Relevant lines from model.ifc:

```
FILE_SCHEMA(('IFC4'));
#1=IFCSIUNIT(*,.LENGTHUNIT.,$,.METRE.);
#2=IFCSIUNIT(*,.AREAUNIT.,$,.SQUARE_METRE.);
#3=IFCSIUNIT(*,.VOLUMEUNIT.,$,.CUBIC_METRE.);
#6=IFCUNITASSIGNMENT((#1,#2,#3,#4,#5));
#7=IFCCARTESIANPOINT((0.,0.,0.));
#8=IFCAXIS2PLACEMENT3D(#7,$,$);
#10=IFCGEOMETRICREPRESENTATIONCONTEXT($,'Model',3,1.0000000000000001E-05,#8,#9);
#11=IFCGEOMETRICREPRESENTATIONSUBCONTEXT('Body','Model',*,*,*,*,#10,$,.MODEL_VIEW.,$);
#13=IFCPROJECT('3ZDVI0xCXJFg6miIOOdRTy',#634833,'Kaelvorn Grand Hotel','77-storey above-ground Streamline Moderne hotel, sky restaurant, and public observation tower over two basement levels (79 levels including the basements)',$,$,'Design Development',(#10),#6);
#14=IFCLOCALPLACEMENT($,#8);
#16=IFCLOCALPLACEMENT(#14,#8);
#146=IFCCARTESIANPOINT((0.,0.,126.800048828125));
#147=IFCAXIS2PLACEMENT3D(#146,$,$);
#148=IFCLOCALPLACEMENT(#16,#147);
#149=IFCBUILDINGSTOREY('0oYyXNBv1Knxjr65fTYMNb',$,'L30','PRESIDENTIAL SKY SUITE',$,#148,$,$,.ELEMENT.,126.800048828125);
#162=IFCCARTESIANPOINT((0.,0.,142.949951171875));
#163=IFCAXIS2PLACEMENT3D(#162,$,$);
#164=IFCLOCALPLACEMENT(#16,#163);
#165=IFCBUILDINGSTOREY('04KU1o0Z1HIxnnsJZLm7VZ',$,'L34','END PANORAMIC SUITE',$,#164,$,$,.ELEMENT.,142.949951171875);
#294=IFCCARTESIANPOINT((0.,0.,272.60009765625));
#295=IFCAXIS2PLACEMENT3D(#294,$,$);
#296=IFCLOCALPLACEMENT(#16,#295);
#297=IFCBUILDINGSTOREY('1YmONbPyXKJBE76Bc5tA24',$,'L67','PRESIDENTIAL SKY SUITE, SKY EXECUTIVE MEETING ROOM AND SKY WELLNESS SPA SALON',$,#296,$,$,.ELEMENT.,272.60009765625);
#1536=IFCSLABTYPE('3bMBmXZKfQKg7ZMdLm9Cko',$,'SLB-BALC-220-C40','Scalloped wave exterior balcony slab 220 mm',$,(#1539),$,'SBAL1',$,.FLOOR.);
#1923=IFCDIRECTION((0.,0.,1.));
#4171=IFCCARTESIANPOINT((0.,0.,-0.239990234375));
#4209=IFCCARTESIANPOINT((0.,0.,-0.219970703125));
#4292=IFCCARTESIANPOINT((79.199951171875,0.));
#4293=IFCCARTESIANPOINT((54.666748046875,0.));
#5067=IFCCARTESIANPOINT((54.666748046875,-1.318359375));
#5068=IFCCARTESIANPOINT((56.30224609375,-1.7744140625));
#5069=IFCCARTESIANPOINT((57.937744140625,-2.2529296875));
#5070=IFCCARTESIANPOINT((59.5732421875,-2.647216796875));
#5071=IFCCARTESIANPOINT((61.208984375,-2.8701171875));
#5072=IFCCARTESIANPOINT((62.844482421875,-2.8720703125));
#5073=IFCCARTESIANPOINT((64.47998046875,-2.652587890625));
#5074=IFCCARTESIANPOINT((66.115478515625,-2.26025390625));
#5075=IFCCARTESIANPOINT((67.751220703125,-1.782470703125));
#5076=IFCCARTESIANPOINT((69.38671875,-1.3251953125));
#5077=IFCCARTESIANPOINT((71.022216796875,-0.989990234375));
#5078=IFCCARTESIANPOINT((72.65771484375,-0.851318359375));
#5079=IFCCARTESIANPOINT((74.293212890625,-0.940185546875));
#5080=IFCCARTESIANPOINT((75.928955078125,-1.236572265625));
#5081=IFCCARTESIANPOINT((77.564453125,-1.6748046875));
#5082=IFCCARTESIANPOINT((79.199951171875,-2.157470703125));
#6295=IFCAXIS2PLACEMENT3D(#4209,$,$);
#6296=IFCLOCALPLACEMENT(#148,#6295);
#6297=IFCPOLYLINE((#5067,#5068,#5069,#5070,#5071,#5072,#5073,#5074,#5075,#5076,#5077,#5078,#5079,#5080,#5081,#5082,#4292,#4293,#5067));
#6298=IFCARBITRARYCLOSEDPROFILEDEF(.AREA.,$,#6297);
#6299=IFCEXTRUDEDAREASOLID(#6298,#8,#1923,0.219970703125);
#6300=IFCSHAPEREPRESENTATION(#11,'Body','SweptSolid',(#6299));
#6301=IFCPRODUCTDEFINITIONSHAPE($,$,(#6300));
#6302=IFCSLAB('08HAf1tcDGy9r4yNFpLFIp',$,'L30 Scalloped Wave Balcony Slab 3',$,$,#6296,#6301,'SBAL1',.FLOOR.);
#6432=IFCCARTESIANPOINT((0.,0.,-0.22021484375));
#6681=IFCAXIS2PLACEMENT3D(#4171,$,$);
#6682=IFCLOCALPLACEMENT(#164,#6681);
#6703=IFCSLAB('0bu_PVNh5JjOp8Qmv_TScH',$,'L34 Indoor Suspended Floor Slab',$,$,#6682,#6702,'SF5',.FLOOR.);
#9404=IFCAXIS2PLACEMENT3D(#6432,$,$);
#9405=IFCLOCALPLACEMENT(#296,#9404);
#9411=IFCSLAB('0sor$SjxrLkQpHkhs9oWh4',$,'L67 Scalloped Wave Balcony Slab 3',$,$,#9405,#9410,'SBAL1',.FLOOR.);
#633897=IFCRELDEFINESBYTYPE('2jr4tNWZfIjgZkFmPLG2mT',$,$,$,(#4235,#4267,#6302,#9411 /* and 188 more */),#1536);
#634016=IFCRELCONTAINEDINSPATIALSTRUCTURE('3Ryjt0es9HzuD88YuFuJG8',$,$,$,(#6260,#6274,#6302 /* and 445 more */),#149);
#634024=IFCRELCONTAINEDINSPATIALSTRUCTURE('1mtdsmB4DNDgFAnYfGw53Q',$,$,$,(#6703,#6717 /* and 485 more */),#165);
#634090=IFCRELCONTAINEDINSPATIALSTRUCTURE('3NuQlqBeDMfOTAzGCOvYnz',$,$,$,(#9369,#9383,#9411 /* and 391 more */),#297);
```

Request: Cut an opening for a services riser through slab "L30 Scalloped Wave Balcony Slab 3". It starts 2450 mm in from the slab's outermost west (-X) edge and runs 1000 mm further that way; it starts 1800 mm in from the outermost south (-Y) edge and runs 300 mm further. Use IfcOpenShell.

```python
import numpy as np
import ifcopenshell
import ifcopenshell.api.feature
import ifcopenshell.api.geometry
import ifcopenshell.api.root
import ifcopenshell.geom
import ifcopenshell.util.placement
import ifcopenshell.util.representation
import ifcopenshell.util.shape
import ifcopenshell.util.unit

model = ifcopenshell.open("model.ifc")
unit_scale = ifcopenshell.util.unit.calculate_unit_scale(model)
settings = ifcopenshell.geom.settings()


def volume(element):
    """Net volume in cubic metres, openings subtracted."""
    shape = ifcopenshell.geom.create_shape(settings, element)
    return ifcopenshell.util.shape.get_volume(shape.geometry)


slab = model.by_guid("08HAf1tcDGy9r4yNFpLFIp")
before = volume(slab)

# Extent in the slab's own axes, in metres. The edges named are its -X and -Y sides.
slab_shape = ifcopenshell.geom.create_shape(settings, slab)
vertices = ifcopenshell.util.shape.get_vertices(slab_shape.geometry)
x_min, y_min, bottom = vertices.min(axis=0)
top = vertices[:, 2].max()

opening = ifcopenshell.api.root.create_entity(model, ifc_class="IfcOpeningElement", name="Services riser opening", predefined_type="OPENING")
context = ifcopenshell.util.representation.get_context(model, "Model", "Body", "MODEL_VIEW")
width, depth = 1, 0.3
outline = [(0.0, 0.0), (width, 0.0), (width, depth), (0.0, depth), (0.0, 0.0)]
# Overshoot both faces by 50 mm so the cut is clean.
shape = ifcopenshell.api.geometry.add_slab_representation(
    model, context=context, depth=top - bottom + 0.1, polyline=outline
)
ifcopenshell.api.geometry.assign_representation(model, product=opening, representation=shape)

matrix = ifcopenshell.util.placement.get_local_placement(slab.ObjectPlacement)
matrix[:, 3] = matrix @ np.append(np.array([x_min + 2.45, y_min + 1.8, bottom - 0.05]) / unit_scale, 1.0)
ifcopenshell.api.geometry.edit_object_placement(model, product=opening, matrix=matrix, is_si=False)
ifcopenshell.api.feature.add_feature(model, feature=opening, element=slab)

after = volume(slab)

print(f"slab volume {before:.3f} -> {after:.3f} m3")

model.write("model_v2.ifc")
```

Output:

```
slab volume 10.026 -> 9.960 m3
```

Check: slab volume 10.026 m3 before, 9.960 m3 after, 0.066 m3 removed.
